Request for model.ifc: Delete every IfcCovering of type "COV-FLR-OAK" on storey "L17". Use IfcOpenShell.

First a look at what the model holds.

```python
import ifcopenshell
import ifcopenshell.util.element

model = ifcopenshell.open("model.ifc")
print(model.schema)
storey = next(s for s in model.by_type("IfcBuildingStorey") if s.Name == "L17")
coverings = [e for e in ifcopenshell.util.element.get_decomposition(storey) if e.is_a("IfcCovering")]
seen = {}
for e in coverings:
    element_type = ifcopenshell.util.element.get_type(e)
    name = element_type.Name if element_type not in (None, e) else None
    seen[name] = seen.get(name, 0) + 1
for name, count in sorted(seen.items(), key=str):
    print(count, "x", name)
```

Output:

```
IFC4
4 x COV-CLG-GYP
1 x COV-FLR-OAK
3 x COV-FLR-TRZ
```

```python
import ifcopenshell
import ifcopenshell.api.root
import ifcopenshell.util.element

model = ifcopenshell.open("model.ifc")

storey = next(s for s in model.by_type("IfcBuildingStorey") if s.Name == "L17")
coverings = [e for e in ifcopenshell.util.element.get_decomposition(storey) if e.is_a("IfcCovering")]
targets = [e for e in coverings if (t := ifcopenshell.util.element.get_type(e)) not in (None, e) and t.Name == "COV-FLR-OAK"]

for e in targets:
    ifcopenshell.api.root.remove_product(model, product=e)
print(len(targets), "removed")

model.write("model_v2.ifc")
```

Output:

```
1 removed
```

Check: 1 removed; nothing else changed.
